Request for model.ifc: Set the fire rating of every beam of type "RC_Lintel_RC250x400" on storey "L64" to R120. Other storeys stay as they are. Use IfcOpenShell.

First a look at what the model holds.

```python
import ifcopenshell
import ifcopenshell.util.element

model = ifcopenshell.open("model.ifc")
print(model.schema)
storey = next(s for s in model.by_type("IfcBuildingStorey") if s.Name == "L64")
beams = [e for e in ifcopenshell.util.element.get_decomposition(storey) if e.is_a("IfcBeam")]
seen = {}
for e in beams:
    element_type = ifcopenshell.util.element.get_type(e)
    key = (element_type.Name if element_type != e and element_type else None, ifcopenshell.util.element.get_pset(e, "Pset_BeamCommon", "FireRating"))
    seen[key] = seen.get(key, 0) + 1
for (name, value), count in sorted(seen.items(), key=str):
    print(count, "x", name, "|", value)
```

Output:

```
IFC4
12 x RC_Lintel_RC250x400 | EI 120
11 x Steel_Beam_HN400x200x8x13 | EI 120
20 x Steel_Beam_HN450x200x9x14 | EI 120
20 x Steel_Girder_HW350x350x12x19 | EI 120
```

```python
import ifcopenshell
import ifcopenshell.api.pset
import ifcopenshell.util.element

model = ifcopenshell.open("model.ifc")

storey = next(s for s in model.by_type("IfcBuildingStorey") if s.Name == "L64")
beams = [e for e in ifcopenshell.util.element.get_decomposition(storey) if e.is_a("IfcBeam")]

count = 0
for e in beams:
    element_type = ifcopenshell.util.element.get_type(e)
    if element_type in (None, e) or element_type.Name != "RC_Lintel_RC250x400":
        continue
    found = ifcopenshell.util.element.get_pset(e, "Pset_BeamCommon", should_inherit=False)
    if found:
        pset = model.by_id(found["id"])
        if len(ifcopenshell.util.element.get_elements_by_pset(pset)) > 1:
            pset = ifcopenshell.api.pset.unshare_pset(model, products=[e], pset=pset)[0]
    else:
        pset = ifcopenshell.api.pset.add_pset(model, product=e, name="Pset_BeamCommon")
    ifcopenshell.api.pset.edit_pset(model, pset=pset, properties={"FireRating": "R120"})
    count += 1

print(count, "beams updated")

model.write("model-out.ifc")
```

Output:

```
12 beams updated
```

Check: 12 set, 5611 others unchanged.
